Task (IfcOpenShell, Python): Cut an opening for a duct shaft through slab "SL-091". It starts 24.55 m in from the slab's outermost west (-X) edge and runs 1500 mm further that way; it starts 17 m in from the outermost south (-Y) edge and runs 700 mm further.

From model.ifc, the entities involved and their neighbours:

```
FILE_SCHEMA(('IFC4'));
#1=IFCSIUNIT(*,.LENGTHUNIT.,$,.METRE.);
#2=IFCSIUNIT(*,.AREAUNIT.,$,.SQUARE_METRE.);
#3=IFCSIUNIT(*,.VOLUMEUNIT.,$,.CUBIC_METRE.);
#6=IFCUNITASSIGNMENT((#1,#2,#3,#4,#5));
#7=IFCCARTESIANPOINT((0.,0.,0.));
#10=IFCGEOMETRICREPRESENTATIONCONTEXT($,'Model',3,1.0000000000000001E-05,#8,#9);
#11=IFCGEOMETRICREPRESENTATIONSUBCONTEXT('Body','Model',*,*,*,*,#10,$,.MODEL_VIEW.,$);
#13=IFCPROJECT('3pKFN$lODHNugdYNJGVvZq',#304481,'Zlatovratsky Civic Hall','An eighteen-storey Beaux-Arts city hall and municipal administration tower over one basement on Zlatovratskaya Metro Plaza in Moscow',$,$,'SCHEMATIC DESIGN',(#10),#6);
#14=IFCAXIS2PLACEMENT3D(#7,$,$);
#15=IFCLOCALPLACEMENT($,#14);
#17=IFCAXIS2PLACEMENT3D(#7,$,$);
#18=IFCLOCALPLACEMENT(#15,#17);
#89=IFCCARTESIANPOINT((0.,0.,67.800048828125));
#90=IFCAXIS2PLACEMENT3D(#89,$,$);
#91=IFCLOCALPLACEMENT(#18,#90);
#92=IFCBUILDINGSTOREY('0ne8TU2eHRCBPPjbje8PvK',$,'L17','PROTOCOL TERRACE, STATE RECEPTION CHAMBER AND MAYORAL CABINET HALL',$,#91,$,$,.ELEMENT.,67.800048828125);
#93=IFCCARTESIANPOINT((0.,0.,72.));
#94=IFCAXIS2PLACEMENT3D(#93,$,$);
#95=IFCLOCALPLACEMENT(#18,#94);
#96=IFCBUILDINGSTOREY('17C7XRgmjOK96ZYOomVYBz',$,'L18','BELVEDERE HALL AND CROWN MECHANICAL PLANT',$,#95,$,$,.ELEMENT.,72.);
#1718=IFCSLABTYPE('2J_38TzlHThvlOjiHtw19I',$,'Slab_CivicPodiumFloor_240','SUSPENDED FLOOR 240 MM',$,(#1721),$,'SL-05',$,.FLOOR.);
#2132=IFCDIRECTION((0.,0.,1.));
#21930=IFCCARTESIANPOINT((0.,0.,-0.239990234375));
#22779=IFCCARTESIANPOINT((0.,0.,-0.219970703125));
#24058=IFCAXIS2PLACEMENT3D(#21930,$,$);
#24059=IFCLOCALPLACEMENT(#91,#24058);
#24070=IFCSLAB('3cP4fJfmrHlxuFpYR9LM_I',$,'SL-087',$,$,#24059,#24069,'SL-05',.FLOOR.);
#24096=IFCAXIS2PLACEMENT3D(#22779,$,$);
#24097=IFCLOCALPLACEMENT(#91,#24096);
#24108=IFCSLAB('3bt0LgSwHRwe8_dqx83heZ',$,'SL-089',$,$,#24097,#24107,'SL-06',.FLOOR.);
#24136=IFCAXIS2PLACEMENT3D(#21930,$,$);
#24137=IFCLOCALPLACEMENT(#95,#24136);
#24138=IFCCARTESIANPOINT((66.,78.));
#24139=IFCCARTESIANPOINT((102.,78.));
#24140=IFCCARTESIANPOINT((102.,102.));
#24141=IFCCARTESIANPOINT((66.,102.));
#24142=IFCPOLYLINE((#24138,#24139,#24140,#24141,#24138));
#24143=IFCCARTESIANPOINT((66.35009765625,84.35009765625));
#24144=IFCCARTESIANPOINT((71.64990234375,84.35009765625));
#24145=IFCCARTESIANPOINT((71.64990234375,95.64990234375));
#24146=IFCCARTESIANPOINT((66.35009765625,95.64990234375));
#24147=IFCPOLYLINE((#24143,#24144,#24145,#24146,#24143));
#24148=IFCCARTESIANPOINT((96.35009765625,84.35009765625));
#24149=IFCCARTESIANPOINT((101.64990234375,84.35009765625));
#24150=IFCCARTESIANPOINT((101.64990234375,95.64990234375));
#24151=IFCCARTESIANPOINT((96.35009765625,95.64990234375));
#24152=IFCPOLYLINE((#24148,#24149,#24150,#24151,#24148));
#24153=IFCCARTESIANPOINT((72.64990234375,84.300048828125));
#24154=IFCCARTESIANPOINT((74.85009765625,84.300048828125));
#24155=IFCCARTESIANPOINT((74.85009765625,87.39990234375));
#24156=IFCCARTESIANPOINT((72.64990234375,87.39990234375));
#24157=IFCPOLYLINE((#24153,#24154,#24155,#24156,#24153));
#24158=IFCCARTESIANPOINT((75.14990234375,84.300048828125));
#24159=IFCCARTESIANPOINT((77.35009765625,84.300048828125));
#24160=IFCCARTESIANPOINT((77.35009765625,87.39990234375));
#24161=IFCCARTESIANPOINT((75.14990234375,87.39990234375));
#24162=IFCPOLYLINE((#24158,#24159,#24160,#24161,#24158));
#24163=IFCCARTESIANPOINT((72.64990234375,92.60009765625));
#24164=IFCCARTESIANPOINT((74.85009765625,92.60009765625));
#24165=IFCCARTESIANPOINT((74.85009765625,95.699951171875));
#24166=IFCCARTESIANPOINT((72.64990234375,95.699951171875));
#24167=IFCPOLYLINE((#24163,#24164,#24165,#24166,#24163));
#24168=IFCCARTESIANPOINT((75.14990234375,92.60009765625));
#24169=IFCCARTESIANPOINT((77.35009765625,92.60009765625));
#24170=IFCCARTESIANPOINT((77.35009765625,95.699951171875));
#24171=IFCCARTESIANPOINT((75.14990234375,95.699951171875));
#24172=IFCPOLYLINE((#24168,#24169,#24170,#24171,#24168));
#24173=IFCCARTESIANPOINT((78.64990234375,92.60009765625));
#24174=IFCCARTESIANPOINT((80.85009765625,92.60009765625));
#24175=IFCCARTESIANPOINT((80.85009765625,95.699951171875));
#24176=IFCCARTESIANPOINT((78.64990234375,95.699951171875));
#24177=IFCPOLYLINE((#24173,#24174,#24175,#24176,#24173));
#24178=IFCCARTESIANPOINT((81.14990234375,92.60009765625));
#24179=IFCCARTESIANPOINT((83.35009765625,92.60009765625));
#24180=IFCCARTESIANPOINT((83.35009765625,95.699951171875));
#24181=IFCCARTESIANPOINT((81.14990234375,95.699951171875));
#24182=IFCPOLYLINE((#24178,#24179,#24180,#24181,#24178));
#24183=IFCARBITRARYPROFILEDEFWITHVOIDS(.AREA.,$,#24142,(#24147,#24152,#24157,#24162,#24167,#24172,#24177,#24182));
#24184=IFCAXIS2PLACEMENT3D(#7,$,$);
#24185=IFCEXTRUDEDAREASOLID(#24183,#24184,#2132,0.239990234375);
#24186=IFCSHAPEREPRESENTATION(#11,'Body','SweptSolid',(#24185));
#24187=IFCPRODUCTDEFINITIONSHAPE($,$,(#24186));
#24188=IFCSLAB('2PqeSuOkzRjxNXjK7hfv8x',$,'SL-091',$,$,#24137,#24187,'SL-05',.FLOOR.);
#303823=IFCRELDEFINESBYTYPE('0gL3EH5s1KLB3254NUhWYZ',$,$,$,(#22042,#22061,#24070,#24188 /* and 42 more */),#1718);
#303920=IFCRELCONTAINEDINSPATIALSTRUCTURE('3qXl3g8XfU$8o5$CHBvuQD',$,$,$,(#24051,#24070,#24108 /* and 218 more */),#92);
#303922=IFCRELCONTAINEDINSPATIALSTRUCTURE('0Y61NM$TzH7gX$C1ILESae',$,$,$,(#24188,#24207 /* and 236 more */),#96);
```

```python
import numpy as np
import ifcopenshell
import ifcopenshell.api.feature
import ifcopenshell.api.geometry
import ifcopenshell.api.root
import ifcopenshell.geom
import ifcopenshell.util.placement
import ifcopenshell.util.representation
import ifcopenshell.util.shape
import ifcopenshell.util.unit

model = ifcopenshell.open("model.ifc")
unit_scale = ifcopenshell.util.unit.calculate_unit_scale(model)
settings = ifcopenshell.geom.settings()


def volume(element):
    """Net volume in cubic metres, openings subtracted."""
    shape = ifcopenshell.geom.create_shape(settings, element)
    return ifcopenshell.util.shape.get_volume(shape.geometry)


slab = model.by_guid("2PqeSuOkzRjxNXjK7hfv8x")
before = volume(slab)

# Extent in the slab's own axes, in metres. The edges named are its -X and -Y sides.
slab_shape = ifcopenshell.geom.create_shape(settings, slab)
vertices = ifcopenshell.util.shape.get_vertices(slab_shape.geometry)
x_min, y_min, bottom = vertices.min(axis=0)
top = vertices[:, 2].max()

opening = ifcopenshell.api.root.create_entity(model, ifc_class="IfcOpeningElement", name="Duct shaft opening", predefined_type="OPENING")
context = ifcopenshell.util.representation.get_context(model, "Model", "Body", "MODEL_VIEW")
width, depth = 1.5, 0.7
outline = [(0.0, 0.0), (width, 0.0), (width, depth), (0.0, depth), (0.0, 0.0)]
# Overshoot both faces by 50 mm so the cut is clean.
shape = ifcopenshell.api.geometry.add_slab_representation(
    model, context=context, depth=top - bottom + 0.1, polyline=outline
)
ifcopenshell.api.geometry.assign_representation(model, product=opening, representation=shape)

matrix = ifcopenshell.util.placement.get_local_placement(slab.ObjectPlacement)
matrix[:, 3] = matrix @ np.append(np.array([x_min + 24.55, y_min + 17, bottom - 0.05]) / unit_scale, 1.0)
ifcopenshell.api.geometry.edit_object_placement(model, product=opening, matrix=matrix, is_si=False)
ifcopenshell.api.feature.add_feature(model, feature=opening, element=slab)

after = volume(slab)

print(f"slab volume {before:.3f} -> {after:.3f} m3")

model.write("model-out.ifc")
```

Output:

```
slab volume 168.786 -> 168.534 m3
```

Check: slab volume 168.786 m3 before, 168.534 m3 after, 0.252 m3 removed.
